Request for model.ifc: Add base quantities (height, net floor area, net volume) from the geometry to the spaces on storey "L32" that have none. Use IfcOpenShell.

First a look at what the model holds.

```python
import ifcopenshell
import ifcopenshell.util.element
import ifcopenshell.util.unit

model = ifcopenshell.open("model.ifc")
print(model.schema)
for unit_type in ("LENGTHUNIT", "AREAUNIT", "VOLUMEUNIT"):
    print(unit_type, ifcopenshell.util.unit.calculate_unit_scale(model, unit_type))
storey = next(s for s in model.by_type("IfcBuildingStorey") if s.Name == "L32")
spaces = [e for e in ifcopenshell.util.element.get_decomposition(storey) if e.is_a("IfcSpace")]
for e in sorted(spaces, key=lambda e: e.id()):
    print(e.id(), e.is_a(), e.Name, list(ifcopenshell.util.element.get_psets(e, qtos_only=True)), sep=" | ")
```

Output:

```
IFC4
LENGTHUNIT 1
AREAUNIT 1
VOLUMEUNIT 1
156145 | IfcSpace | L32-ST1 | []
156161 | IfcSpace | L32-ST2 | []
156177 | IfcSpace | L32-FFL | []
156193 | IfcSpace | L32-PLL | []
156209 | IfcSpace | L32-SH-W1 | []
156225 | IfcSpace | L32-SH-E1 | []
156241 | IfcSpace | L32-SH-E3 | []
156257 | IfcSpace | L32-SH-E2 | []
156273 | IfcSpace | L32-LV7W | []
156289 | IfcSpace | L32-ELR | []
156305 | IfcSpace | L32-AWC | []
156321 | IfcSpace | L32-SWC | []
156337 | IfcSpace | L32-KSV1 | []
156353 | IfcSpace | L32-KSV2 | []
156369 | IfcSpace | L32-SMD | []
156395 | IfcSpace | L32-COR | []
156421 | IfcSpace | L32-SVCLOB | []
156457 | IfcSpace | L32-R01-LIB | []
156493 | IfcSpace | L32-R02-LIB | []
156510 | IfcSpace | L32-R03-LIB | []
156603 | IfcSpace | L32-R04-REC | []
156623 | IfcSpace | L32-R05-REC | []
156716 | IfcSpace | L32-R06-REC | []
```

```python
import ifcopenshell
import ifcopenshell.api.pset
import ifcopenshell.geom
import ifcopenshell.util.element
import ifcopenshell.util.shape
import ifcopenshell.util.unit

model = ifcopenshell.open("model.ifc")
unit_scale = ifcopenshell.util.unit.calculate_unit_scale(model)
area_scale = ifcopenshell.util.unit.calculate_unit_scale(model, "AREAUNIT")
volume_scale = ifcopenshell.util.unit.calculate_unit_scale(model, "VOLUMEUNIT")
settings = ifcopenshell.geom.settings()

storey = next(s for s in model.by_type("IfcBuildingStorey") if s.Name == "L32")
spaces = [e for e in ifcopenshell.util.element.get_decomposition(storey) if e.is_a("IfcSpace")]

for e in sorted(spaces, key=lambda e: e.id()):
    if ifcopenshell.util.element.get_psets(e, qtos_only=True, should_inherit=False):
        continue
    # Geometry comes back in metres, in the element's own axes.
    shape = ifcopenshell.geom.create_shape(settings, e)
    values = {
        "Height": ifcopenshell.util.shape.get_z(shape.geometry) / unit_scale,
        "NetFloorArea": ifcopenshell.util.shape.get_footprint_area(shape.geometry) / area_scale,
        "NetVolume": ifcopenshell.util.shape.get_volume(shape.geometry) / volume_scale,
    }
    qto = ifcopenshell.api.pset.add_qto(model, product=e, name="Qto_SpaceBaseQuantities")
    ifcopenshell.api.pset.edit_qto(model, qto=qto, properties=values)
    print(e.id(), {k: round(v, 3) for k, v in values.items()})

model.write("model_v2.ifc")
```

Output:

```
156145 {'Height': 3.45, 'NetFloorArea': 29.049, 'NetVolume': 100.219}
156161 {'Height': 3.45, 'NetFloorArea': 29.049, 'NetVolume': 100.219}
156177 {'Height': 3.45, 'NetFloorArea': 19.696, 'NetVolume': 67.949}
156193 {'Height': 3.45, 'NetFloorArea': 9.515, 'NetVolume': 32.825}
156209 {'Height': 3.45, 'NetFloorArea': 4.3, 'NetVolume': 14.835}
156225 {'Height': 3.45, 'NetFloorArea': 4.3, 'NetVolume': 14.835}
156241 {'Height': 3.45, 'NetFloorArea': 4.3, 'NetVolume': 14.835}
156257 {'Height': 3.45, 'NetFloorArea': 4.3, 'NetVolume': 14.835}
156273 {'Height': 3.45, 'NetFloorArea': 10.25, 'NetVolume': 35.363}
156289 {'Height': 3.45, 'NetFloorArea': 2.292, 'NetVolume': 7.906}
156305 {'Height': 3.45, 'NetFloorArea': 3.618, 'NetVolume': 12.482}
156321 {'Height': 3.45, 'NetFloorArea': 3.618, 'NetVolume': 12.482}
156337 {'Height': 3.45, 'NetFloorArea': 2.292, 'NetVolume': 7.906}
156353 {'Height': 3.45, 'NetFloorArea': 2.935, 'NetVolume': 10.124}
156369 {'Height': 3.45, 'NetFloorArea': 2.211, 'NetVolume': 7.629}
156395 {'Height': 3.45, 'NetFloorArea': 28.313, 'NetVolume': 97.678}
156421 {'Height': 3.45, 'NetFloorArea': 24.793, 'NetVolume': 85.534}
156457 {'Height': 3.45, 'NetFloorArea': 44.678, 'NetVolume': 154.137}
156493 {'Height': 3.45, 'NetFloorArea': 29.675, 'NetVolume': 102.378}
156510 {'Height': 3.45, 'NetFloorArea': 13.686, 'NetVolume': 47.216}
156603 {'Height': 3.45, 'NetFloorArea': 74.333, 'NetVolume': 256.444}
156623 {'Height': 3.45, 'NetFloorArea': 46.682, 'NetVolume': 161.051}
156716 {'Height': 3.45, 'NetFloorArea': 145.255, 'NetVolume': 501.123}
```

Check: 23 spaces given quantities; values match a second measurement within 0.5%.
